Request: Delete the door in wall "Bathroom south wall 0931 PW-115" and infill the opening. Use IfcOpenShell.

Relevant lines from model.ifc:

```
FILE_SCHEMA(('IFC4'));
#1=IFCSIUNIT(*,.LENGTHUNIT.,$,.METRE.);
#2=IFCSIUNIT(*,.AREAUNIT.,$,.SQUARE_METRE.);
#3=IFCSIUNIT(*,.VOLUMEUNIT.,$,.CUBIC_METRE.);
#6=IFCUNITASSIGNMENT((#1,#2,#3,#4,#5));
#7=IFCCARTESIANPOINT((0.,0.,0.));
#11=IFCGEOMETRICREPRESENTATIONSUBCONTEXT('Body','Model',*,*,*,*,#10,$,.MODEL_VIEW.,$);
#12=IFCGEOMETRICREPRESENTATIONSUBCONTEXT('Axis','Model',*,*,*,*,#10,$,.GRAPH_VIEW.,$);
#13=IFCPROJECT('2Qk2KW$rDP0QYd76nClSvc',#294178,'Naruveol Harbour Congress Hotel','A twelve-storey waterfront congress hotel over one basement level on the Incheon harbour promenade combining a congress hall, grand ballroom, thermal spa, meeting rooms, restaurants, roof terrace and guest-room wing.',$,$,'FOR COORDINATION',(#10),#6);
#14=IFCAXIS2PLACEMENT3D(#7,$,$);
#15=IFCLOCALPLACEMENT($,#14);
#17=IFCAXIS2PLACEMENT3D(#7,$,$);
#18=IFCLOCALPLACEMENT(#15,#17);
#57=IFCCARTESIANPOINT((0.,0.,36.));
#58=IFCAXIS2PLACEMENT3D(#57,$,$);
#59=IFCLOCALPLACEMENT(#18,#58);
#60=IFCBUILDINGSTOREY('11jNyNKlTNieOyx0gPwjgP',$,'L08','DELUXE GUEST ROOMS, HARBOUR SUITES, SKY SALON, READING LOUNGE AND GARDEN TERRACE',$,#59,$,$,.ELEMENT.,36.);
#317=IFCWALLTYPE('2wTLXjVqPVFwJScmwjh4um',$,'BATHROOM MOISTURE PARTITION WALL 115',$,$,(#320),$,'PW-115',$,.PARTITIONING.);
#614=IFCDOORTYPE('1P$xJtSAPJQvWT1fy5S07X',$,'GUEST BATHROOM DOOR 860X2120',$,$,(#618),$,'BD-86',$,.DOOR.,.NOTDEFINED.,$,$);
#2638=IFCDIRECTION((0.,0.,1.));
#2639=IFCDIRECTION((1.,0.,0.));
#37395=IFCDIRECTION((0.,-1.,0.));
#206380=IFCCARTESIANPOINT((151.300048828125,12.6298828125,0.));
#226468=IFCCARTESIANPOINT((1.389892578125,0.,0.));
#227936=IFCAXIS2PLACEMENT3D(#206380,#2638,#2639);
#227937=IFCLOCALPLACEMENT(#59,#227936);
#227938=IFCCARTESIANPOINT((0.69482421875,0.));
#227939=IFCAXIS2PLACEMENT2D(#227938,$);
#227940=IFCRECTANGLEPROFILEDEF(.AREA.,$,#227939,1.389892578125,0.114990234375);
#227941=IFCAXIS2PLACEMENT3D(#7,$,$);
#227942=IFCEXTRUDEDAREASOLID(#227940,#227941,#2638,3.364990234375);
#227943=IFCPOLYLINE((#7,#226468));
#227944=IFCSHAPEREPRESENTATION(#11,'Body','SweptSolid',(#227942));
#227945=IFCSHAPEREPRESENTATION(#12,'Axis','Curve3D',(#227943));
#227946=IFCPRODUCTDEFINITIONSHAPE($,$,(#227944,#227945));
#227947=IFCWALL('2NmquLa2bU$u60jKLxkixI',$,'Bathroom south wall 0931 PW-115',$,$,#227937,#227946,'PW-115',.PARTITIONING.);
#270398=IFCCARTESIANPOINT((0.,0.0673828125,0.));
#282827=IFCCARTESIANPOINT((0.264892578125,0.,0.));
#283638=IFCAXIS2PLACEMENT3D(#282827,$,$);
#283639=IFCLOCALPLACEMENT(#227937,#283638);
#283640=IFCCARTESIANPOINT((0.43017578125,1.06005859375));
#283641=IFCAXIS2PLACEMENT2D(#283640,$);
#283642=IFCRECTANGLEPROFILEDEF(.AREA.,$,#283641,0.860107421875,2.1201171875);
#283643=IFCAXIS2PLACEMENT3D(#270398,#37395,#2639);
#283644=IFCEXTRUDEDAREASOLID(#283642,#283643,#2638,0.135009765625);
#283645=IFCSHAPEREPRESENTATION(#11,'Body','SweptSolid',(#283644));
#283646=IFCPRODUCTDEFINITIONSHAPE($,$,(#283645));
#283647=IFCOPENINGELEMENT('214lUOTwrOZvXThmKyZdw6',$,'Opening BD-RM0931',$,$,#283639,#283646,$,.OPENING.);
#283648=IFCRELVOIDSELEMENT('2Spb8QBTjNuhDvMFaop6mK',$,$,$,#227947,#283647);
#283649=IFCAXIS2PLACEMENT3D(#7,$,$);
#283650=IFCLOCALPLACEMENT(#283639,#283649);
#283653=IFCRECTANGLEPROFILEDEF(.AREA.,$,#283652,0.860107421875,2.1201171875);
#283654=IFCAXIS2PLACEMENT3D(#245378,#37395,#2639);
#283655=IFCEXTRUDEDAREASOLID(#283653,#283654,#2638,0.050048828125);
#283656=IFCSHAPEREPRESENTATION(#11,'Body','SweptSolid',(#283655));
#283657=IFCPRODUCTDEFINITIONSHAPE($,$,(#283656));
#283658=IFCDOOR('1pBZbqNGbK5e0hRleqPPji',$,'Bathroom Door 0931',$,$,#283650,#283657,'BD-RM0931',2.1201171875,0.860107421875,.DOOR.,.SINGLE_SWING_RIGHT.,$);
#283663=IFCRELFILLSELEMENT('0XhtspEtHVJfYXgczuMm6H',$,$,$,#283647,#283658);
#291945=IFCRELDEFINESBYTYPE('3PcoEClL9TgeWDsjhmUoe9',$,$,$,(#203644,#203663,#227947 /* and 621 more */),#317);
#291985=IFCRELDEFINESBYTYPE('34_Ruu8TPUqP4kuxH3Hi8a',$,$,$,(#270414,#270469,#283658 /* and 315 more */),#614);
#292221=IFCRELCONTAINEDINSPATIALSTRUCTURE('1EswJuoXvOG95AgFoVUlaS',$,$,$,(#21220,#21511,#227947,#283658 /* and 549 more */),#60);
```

```python
import ifcopenshell
import ifcopenshell.api.feature
import ifcopenshell.api.root
import ifcopenshell.geom
import ifcopenshell.util.shape

model = ifcopenshell.open("model.ifc")
settings = ifcopenshell.geom.settings()


def volume(element):
    """Net volume in cubic metres, openings subtracted."""
    shape = ifcopenshell.geom.create_shape(settings, element)
    return ifcopenshell.util.shape.get_volume(shape.geometry)


door = model.by_guid("1pBZbqNGbK5e0hRleqPPji")
opening = door.FillsVoids[0].RelatingOpeningElement
wall = opening.VoidsElements[0].RelatingBuildingElement
before = volume(wall)

ifcopenshell.api.root.remove_product(model, product=door)
ifcopenshell.api.feature.remove_feature(model, feature=opening)

after = volume(wall)

print(f"wall volume {before:.3f} -> {after:.3f} m3")

model.write("model_edited.ifc")
```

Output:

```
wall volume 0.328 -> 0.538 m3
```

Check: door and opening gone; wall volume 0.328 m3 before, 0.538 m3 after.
